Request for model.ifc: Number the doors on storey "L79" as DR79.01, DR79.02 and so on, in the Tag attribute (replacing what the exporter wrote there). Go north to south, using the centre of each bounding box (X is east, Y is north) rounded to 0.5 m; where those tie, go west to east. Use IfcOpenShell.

First a look at what the model holds.

```python
import ifcopenshell
import ifcopenshell.util.element
import ifcopenshell.util.placement

model = ifcopenshell.open("model.ifc")
print(model.schema)
storey = next(s for s in model.by_type("IfcBuildingStorey") if s.Name == "L79")
doors = [e for e in ifcopenshell.util.element.get_decomposition(storey) if e.is_a("IfcDoor")]
for e in sorted(doors, key=lambda e: e.id()):
    origin = ifcopenshell.util.placement.get_local_placement(e.ObjectPlacement)[:3, 3]
    print(e.id(), e.Tag, e.Name, origin.round(2) + 0.0, sep=" | ")
```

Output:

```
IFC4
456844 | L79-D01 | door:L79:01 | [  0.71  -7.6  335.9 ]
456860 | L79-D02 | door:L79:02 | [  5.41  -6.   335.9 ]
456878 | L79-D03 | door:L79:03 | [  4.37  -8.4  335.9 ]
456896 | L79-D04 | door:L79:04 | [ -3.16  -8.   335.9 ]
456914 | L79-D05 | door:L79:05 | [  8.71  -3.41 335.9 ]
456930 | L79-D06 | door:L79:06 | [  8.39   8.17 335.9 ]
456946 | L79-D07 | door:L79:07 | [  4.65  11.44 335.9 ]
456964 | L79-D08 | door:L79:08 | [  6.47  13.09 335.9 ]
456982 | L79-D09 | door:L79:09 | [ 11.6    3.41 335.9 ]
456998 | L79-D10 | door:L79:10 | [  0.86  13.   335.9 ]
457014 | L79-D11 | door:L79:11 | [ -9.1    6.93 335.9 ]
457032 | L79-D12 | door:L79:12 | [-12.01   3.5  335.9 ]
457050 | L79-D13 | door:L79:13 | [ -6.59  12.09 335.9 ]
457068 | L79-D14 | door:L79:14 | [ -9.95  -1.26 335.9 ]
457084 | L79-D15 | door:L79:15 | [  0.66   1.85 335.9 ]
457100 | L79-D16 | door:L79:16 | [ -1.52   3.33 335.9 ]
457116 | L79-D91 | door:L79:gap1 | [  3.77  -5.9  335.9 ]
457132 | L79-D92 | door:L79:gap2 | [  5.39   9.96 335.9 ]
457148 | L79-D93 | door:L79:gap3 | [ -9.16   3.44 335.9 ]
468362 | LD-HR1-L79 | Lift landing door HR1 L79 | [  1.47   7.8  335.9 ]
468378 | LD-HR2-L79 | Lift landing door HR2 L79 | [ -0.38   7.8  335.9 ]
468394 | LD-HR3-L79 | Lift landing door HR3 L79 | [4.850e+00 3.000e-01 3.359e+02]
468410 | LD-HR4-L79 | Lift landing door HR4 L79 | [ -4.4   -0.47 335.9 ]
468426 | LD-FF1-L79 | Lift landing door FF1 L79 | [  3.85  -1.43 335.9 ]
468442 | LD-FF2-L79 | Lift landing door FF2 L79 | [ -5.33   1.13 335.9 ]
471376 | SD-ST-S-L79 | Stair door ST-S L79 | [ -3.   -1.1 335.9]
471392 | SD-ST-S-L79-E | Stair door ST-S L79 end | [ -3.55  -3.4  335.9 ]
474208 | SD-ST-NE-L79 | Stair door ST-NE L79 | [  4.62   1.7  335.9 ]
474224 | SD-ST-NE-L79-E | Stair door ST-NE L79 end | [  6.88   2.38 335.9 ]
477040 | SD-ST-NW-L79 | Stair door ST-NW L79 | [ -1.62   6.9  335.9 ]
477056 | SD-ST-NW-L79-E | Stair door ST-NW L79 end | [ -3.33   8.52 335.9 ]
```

```python
import ifcopenshell
import ifcopenshell.geom
import ifcopenshell.util.element
import ifcopenshell.util.shape

model = ifcopenshell.open("model.ifc")
settings = ifcopenshell.geom.settings()
settings.set("use-world-coords", True)


def centre(element):
    shape = ifcopenshell.geom.create_shape(settings, element)
    return ifcopenshell.util.shape.get_bbox_centroid(shape.geometry)


storey = next(s for s in model.by_type("IfcBuildingStorey") if s.Name == "L79")
doors = [e for e in ifcopenshell.util.element.get_decomposition(storey) if e.is_a("IfcDoor")]

# Insertion points can sit at a corner or the storey origin, so sort by the geometry (in metres).
centres = {e: centre(e) for e in doors}
doors.sort(key=lambda e: (-round(centres[e][1] / 0.5), centres[e][0]))

for i, e in enumerate(doors, start=1):
    number = f"DR79.{i:02d}"
    e.Tag = number
    print(e.id(), number)

model.write("model_rev.ifc")
```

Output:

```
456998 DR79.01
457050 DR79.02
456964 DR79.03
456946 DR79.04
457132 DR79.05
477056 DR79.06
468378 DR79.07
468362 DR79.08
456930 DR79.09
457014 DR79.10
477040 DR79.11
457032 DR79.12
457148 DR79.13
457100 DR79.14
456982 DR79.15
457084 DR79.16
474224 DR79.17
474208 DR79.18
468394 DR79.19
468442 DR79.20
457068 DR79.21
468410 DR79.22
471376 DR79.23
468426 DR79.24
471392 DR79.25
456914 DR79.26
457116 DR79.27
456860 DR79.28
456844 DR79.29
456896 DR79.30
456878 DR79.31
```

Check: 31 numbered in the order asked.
